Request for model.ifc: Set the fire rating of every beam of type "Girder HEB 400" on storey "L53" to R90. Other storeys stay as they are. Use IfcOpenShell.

First a look at what the model holds.

```python
import ifcopenshell
import ifcopenshell.util.element

model = ifcopenshell.open("model.ifc")
print(model.schema)
storey = next(s for s in model.by_type("IfcBuildingStorey") if s.Name == "L53")
beams = [e for e in ifcopenshell.util.element.get_decomposition(storey) if e.is_a("IfcBeam")]
seen = {}
for e in beams:
    element_type = ifcopenshell.util.element.get_type(e)
    key = (element_type.Name if element_type != e and element_type else None, ifcopenshell.util.element.get_pset(e, "Pset_BeamCommon", "FireRating"))
    seen[key] = seen.get(key, 0) + 1
for (name, value), count in sorted(seen.items(), key=str):
    print(count, "x", name, "|", value)
```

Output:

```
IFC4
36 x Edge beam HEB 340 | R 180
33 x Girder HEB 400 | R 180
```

```python
import ifcopenshell
import ifcopenshell.api.pset
import ifcopenshell.util.element

model = ifcopenshell.open("model.ifc")

storey = next(s for s in model.by_type("IfcBuildingStorey") if s.Name == "L53")
beams = [e for e in ifcopenshell.util.element.get_decomposition(storey) if e.is_a("IfcBeam")]

count = 0
for e in beams:
    element_type = ifcopenshell.util.element.get_type(e)
    if element_type in (None, e) or element_type.Name != "Girder HEB 400":
        continue
    found = ifcopenshell.util.element.get_pset(e, "Pset_BeamCommon", should_inherit=False)
    if found:
        pset = model.by_id(found["id"])
        if len(ifcopenshell.util.element.get_elements_by_pset(pset)) > 1:
            pset = ifcopenshell.api.pset.unshare_pset(model, products=[e], pset=pset)[0]
    else:
        pset = ifcopenshell.api.pset.add_pset(model, product=e, name="Pset_BeamCommon")
    ifcopenshell.api.pset.edit_pset(model, pset=pset, properties={"FireRating": "R90"})
    count += 1

print(count, "beams updated")

model.write("model_updated.ifc")
```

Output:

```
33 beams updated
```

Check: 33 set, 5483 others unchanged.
